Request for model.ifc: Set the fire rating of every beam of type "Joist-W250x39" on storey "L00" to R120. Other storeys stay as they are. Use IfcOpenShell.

First a look at what the model holds.

```python
import ifcopenshell
import ifcopenshell.util.element

model = ifcopenshell.open("model.ifc")
print(model.schema)
storey = next(s for s in model.by_type("IfcBuildingStorey") if s.Name == "L00")
beams = [e for e in ifcopenshell.util.element.get_decomposition(storey) if e.is_a("IfcBeam")]
seen = {}
for e in beams:
    element_type = ifcopenshell.util.element.get_type(e)
    key = (element_type.Name if element_type != e and element_type else None, ifcopenshell.util.element.get_pset(e, "Pset_BeamCommon", "FireRating"))
    seen[key] = seen.get(key, 0) + 1
for (name, value), count in sorted(seen.items(), key=str):
    print(count, "x", name, "|", value)
```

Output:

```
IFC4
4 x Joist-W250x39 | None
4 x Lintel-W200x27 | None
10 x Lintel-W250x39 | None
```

```python
import ifcopenshell
import ifcopenshell.api.pset
import ifcopenshell.util.element

model = ifcopenshell.open("model.ifc")

storey = next(s for s in model.by_type("IfcBuildingStorey") if s.Name == "L00")
beams = [e for e in ifcopenshell.util.element.get_decomposition(storey) if e.is_a("IfcBeam")]

count = 0
for e in beams:
    element_type = ifcopenshell.util.element.get_type(e)
    if element_type in (None, e) or element_type.Name != "Joist-W250x39":
        continue
    # add_pset returns the element's existing set when there is one.
    pset = ifcopenshell.api.pset.add_pset(model, product=e, name="Pset_BeamCommon")
    ifcopenshell.api.pset.edit_pset(model, pset=pset, properties={"FireRating": "R120"})
    count += 1

print(count, "beams updated")

model.write("model_v2.ifc")
```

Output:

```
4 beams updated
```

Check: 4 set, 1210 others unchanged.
